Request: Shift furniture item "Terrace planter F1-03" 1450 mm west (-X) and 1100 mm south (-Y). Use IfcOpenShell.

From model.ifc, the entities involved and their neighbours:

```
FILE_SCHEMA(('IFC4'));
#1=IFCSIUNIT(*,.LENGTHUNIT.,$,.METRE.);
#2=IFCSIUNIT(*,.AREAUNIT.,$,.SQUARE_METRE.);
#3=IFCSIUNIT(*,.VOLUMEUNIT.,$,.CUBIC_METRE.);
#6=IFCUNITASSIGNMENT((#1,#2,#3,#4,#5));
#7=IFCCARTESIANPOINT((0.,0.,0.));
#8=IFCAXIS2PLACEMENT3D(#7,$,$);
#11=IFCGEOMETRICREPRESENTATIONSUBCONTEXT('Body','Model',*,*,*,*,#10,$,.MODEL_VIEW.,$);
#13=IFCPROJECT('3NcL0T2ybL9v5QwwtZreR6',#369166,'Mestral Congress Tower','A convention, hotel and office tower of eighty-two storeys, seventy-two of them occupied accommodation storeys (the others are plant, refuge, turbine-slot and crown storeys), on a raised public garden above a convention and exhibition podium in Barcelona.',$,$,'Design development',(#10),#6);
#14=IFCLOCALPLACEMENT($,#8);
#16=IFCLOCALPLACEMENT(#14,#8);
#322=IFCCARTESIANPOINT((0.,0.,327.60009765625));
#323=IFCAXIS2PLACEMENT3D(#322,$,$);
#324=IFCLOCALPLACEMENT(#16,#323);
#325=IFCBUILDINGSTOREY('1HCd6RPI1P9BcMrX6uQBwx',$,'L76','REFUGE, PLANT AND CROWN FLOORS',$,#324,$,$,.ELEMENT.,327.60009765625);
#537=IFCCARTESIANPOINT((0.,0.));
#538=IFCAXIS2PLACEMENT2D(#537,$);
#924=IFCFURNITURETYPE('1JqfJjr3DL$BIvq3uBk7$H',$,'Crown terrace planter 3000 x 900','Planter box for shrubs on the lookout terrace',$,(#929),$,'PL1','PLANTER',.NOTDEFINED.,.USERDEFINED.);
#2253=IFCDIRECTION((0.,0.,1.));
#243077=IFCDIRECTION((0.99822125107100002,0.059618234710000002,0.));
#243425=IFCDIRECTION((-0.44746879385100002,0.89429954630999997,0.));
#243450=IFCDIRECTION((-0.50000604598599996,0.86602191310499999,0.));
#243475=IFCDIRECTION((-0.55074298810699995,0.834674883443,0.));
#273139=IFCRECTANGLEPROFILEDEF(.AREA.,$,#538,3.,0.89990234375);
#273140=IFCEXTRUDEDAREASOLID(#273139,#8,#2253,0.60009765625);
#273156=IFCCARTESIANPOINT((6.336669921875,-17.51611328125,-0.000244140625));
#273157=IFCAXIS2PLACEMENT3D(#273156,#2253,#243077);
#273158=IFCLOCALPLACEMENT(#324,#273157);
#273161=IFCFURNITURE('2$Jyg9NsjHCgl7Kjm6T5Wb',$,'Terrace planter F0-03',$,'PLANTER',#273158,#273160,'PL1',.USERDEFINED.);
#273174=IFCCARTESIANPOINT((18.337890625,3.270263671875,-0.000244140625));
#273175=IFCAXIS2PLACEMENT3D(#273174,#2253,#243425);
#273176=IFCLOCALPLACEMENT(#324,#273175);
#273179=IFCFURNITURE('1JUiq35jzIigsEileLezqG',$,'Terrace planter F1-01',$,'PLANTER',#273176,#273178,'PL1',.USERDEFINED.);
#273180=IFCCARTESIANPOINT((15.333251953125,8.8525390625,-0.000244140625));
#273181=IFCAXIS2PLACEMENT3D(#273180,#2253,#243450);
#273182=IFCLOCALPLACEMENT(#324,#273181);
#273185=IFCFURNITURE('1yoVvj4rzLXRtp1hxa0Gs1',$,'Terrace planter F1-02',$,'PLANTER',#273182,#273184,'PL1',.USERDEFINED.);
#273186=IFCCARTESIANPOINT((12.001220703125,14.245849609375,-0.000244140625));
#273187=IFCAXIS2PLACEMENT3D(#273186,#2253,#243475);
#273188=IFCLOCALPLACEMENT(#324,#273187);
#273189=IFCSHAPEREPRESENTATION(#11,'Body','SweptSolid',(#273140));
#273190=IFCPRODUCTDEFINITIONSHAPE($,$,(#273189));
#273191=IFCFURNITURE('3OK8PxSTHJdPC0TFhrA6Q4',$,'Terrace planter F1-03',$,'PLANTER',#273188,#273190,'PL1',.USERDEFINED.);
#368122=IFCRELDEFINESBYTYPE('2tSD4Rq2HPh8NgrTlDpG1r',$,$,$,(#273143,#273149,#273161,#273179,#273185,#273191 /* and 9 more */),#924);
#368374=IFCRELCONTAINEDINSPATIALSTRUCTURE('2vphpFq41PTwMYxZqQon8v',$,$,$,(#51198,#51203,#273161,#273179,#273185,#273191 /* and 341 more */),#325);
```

```python
import ifcopenshell
import ifcopenshell.api.geometry
import ifcopenshell.util.placement
import ifcopenshell.util.unit

model = ifcopenshell.open("model.ifc")
unit_scale = ifcopenshell.util.unit.calculate_unit_scale(model)

item = model.by_guid("3OK8PxSTHJdPC0TFhrA6Q4")
matrix = ifcopenshell.util.placement.get_local_placement(item.ObjectPlacement)
matrix[0, 3] -= 1.45 / unit_scale
matrix[1, 3] -= 1.1 / unit_scale
ifcopenshell.api.geometry.edit_object_placement(model, product=item, matrix=matrix, is_si=False)

print(ifcopenshell.util.placement.get_local_placement(item.ObjectPlacement).round(3) + 0.0)

model.write("model_updated.ifc")
```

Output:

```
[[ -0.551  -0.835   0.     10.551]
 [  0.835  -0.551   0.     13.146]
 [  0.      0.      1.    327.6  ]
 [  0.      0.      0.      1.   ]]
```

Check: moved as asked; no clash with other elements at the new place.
